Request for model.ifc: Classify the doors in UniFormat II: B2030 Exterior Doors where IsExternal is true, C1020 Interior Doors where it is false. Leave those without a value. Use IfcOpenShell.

First a look at what the model holds.

```python
import ifcopenshell
import ifcopenshell.util.element

model = ifcopenshell.open("model.ifc")
print(model.schema)
print("classifications:", [c.Name for c in model.by_type("IfcClassification")])
values = [ifcopenshell.util.element.get_pset(e, "Pset_DoorCommon", "IsExternal") for e in model.by_type("IfcDoor")]
for value in (True, False, None):
    print("IsExternal", value, values.count(value))
```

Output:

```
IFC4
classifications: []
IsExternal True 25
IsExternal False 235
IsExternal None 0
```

```python
import ifcopenshell
import ifcopenshell.api.classification
import ifcopenshell.util.element

model = ifcopenshell.open("model.ifc")

system = ifcopenshell.api.classification.add_classification(model, classification="UniFormat II")

doors = model.by_type("IfcDoor")
external = {e: ifcopenshell.util.element.get_pset(e, "Pset_DoorCommon", "IsExternal") for e in doors}
for flag, code, name in ((True, "B2030", "Exterior Doors"), (False, "C1020", "Interior Doors")):
    products = [e for e in doors if external[e] is flag]
    ifcopenshell.api.classification.add_reference(
        model, products=products, classification=system, identification=code, name=name
    )
    print(code, len(products))

model.write("model_updated.ifc")
```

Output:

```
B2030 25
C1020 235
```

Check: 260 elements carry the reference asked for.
